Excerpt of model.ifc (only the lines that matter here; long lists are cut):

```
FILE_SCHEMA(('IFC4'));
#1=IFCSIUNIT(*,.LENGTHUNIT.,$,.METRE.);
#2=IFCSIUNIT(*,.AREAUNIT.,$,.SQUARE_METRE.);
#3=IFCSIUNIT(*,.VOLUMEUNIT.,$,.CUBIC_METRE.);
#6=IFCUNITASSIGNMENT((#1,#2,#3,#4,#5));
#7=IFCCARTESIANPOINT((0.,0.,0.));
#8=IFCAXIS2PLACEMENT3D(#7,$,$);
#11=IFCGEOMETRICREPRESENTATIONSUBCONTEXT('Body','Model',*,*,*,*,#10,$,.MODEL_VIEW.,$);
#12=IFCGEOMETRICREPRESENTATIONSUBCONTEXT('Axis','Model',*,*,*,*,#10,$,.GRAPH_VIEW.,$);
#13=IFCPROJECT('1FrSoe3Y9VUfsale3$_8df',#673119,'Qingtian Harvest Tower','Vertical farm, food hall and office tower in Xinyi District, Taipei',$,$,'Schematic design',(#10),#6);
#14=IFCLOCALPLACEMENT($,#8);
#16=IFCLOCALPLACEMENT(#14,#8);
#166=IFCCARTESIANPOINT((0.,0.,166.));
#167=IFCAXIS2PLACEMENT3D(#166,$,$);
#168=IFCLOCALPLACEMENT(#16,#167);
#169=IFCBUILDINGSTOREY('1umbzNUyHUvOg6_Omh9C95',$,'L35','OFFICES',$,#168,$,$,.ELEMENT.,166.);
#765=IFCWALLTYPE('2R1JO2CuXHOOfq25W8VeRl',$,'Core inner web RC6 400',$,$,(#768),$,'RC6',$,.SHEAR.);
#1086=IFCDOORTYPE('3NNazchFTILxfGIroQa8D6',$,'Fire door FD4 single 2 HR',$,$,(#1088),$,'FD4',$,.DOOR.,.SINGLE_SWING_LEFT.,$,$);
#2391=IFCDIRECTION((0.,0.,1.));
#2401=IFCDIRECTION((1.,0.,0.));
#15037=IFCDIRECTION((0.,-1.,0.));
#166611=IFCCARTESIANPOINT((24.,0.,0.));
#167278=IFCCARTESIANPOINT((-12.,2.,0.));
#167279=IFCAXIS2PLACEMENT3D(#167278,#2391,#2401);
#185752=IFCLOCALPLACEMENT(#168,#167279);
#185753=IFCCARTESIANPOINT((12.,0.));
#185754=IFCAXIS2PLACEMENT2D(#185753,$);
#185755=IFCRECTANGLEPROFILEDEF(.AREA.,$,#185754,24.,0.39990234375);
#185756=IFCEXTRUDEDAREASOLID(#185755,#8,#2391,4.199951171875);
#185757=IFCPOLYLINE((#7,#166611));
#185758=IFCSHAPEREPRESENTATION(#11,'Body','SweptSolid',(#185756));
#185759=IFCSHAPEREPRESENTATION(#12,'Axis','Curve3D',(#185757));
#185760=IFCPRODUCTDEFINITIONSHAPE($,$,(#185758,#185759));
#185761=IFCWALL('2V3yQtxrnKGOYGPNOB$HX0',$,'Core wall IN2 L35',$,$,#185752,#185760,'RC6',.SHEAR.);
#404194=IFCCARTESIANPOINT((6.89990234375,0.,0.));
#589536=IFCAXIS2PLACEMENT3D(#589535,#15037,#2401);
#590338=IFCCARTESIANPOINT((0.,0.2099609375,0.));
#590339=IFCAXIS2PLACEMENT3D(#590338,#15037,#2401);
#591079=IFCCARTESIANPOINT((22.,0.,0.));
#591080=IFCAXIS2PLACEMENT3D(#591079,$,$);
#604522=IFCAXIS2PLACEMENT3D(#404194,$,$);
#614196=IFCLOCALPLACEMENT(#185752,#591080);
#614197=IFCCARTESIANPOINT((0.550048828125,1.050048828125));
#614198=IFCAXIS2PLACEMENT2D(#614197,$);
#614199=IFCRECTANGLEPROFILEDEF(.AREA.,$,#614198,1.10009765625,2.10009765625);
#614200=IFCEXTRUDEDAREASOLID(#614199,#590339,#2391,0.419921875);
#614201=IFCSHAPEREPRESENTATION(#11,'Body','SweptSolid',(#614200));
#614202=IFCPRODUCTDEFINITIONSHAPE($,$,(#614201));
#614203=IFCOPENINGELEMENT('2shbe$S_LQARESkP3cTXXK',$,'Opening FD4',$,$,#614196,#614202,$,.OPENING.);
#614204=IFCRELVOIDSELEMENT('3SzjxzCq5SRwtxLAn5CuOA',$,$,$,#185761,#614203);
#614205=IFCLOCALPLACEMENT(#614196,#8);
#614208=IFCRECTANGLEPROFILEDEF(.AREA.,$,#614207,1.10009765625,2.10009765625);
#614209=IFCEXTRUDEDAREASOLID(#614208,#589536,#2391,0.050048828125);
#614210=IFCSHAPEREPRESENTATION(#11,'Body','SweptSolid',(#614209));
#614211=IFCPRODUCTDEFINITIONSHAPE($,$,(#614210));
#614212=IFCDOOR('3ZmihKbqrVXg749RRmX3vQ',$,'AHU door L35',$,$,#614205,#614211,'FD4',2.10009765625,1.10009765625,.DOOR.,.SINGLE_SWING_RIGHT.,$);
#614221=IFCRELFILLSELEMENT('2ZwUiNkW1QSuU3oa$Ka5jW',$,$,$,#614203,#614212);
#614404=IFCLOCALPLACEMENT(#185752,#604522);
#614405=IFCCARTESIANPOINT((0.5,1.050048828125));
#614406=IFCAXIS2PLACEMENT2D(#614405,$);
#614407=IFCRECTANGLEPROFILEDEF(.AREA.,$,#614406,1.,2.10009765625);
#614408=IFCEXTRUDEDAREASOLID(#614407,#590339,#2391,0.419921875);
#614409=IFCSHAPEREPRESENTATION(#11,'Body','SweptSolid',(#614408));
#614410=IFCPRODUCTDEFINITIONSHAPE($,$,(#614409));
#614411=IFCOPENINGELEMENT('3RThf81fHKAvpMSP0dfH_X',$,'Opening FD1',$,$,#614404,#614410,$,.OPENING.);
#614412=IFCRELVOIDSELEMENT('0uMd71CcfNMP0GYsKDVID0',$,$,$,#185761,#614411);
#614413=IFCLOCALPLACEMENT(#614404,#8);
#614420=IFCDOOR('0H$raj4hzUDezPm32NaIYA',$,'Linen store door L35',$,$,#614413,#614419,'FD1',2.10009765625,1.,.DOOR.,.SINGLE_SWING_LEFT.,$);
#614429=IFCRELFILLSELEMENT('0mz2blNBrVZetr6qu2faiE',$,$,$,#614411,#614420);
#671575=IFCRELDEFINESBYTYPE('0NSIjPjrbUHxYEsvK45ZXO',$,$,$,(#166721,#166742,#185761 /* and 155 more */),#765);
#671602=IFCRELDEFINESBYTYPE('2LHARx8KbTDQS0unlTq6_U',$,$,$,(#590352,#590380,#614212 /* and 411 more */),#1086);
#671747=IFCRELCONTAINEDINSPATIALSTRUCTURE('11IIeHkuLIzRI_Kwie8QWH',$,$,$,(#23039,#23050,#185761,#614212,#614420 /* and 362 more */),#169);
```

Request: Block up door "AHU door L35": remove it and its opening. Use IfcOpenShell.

```python
import ifcopenshell
import ifcopenshell.api.feature
import ifcopenshell.api.root
import ifcopenshell.geom
import ifcopenshell.util.shape

model = ifcopenshell.open("model.ifc")
settings = ifcopenshell.geom.settings()


def volume(element):
    """Net volume in cubic metres, openings subtracted."""
    shape = ifcopenshell.geom.create_shape(settings, element)
    return ifcopenshell.util.shape.get_volume(shape.geometry)


door = model.by_guid("3ZmihKbqrVXg749RRmX3vQ")
opening = door.FillsVoids[0].RelatingOpeningElement
wall = opening.VoidsElements[0].RelatingBuildingElement
before = volume(wall)

ifcopenshell.api.root.remove_product(model, product=door)
ifcopenshell.api.feature.remove_feature(model, feature=opening)

after = volume(wall)

print(f"wall volume {before:.3f} -> {after:.3f} m3")

model.write("model_updated.ifc")
```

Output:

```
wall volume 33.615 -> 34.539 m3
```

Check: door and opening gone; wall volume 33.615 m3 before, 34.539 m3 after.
